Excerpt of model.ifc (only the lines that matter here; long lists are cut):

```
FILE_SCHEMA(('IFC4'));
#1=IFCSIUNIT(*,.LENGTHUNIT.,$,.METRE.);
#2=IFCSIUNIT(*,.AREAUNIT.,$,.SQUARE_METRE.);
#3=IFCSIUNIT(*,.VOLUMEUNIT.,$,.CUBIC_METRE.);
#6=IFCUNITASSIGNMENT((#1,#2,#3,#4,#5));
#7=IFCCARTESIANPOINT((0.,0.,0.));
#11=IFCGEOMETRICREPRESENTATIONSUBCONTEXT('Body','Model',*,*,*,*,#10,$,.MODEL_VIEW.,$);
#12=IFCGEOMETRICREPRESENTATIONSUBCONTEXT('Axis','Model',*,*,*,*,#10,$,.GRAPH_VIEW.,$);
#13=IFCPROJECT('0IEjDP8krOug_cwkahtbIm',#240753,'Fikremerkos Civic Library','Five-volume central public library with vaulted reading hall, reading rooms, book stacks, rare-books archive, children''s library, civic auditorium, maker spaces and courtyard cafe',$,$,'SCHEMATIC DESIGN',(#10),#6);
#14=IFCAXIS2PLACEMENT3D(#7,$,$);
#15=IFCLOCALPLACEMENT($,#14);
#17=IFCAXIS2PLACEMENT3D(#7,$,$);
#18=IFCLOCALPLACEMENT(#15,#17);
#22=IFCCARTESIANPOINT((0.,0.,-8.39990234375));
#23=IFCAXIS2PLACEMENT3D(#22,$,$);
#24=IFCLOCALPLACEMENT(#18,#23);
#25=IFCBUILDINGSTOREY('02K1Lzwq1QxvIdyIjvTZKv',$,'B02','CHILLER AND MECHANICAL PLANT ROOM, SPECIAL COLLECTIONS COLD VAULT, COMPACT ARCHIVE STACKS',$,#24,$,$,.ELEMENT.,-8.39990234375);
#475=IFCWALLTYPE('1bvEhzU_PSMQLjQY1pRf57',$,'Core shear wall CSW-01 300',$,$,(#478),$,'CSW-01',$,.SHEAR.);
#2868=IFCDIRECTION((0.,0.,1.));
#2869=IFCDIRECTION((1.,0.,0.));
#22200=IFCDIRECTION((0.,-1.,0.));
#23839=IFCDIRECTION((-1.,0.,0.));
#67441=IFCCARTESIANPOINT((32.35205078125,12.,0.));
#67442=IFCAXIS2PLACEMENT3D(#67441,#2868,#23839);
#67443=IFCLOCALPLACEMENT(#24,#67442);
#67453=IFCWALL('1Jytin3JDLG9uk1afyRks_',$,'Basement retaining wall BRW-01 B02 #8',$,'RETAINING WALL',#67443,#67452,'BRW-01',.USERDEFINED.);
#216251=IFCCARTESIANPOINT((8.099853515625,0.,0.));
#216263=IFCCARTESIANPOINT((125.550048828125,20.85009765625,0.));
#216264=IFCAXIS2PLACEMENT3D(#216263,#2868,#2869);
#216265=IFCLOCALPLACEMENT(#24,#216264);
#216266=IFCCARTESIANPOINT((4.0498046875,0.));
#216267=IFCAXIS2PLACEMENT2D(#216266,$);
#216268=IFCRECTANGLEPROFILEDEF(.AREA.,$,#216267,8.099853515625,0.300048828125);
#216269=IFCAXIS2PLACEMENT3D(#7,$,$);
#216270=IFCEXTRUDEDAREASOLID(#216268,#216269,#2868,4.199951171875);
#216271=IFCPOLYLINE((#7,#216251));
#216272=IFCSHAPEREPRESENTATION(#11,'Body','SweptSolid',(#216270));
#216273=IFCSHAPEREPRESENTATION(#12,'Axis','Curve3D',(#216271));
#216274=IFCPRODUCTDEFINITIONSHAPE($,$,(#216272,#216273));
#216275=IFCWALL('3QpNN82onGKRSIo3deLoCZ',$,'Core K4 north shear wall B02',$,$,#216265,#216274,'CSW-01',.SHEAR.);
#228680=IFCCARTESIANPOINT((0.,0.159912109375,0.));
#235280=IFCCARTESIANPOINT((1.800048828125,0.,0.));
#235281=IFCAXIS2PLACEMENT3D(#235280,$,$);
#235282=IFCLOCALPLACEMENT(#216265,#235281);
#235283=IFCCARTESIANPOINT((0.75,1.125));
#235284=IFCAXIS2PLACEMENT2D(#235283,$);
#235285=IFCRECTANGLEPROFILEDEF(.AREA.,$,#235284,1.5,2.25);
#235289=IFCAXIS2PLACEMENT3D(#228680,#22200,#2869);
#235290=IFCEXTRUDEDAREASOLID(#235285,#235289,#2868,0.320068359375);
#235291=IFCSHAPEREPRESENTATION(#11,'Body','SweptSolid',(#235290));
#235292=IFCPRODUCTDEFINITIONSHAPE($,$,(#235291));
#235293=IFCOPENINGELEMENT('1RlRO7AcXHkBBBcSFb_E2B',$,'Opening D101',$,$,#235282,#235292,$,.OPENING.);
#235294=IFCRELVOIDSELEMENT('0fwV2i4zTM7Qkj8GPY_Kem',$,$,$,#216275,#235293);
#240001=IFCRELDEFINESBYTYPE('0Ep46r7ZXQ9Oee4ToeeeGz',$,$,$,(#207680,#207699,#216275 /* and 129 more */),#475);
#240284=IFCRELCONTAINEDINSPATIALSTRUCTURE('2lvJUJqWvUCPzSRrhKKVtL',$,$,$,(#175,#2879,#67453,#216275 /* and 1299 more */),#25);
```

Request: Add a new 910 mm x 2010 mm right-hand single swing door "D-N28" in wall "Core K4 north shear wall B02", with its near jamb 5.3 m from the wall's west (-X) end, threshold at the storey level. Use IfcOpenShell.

```python
import numpy as np
import ifcopenshell
import ifcopenshell.api.feature
import ifcopenshell.api.geometry
import ifcopenshell.api.root
import ifcopenshell.api.spatial
import ifcopenshell.geom
import ifcopenshell.util.element
import ifcopenshell.util.placement
import ifcopenshell.util.representation
import ifcopenshell.util.shape
import ifcopenshell.util.unit

model = ifcopenshell.open("model.ifc")
unit_scale = ifcopenshell.util.unit.calculate_unit_scale(model)
settings = ifcopenshell.geom.settings()


def volume(element):
    """Net volume in cubic metres, openings subtracted."""
    shape = ifcopenshell.geom.create_shape(settings, element)
    return ifcopenshell.util.shape.get_volume(shape.geometry)


wall = model.by_guid("3QpNN82onGKRSIo3deLoCZ")
storey = ifcopenshell.util.element.get_container(wall, ifc_class="IfcBuildingStorey")
context = ifcopenshell.util.representation.get_context(model, "Model", "Body", "MODEL_VIEW")
before = volume(wall)

width, height, from_end, sill = 0.91, 2.01, 5.3, 0.0  # metres

# The wall runs along its own X axis, and the end named is its -X end.
wall_shape = ifcopenshell.geom.create_shape(settings, wall)
x, y, z = ifcopenshell.util.shape.get_vertices(wall_shape.geometry).T
start = x.min() + from_end
face, thickness = float(y.min()), float(y.max() - y.min())
wall_matrix = ifcopenshell.util.placement.get_local_placement(wall.ObjectPlacement)
level = ifcopenshell.util.placement.get_local_placement(storey.ObjectPlacement)[2, 3]


def in_wall(x, y):
    """Placement at x, y metres in the wall's axes, at sill height."""
    matrix = wall_matrix.copy()
    matrix[:, 3] = wall_matrix @ np.array([x / unit_scale, y / unit_scale, 0.0, 1.0])
    matrix[2, 3] = level + sill / unit_scale
    return matrix


# Opening: a box that overshoots both wall faces by 50 mm.
opening = ifcopenshell.api.root.create_entity(model, ifc_class="IfcOpeningElement", predefined_type="OPENING")
box = ifcopenshell.api.geometry.add_wall_representation(
    model, context=context, length=width, height=height, thickness=thickness + 0.1
)
ifcopenshell.api.geometry.assign_representation(model, product=opening, representation=box)
ifcopenshell.api.geometry.edit_object_placement(model, product=opening, matrix=in_wall(start, face - 0.05), is_si=False)
ifcopenshell.api.feature.add_feature(model, feature=opening, element=wall)

door = ifcopenshell.api.root.create_entity(model, ifc_class="IfcDoor", name="D-N28", predefined_type="DOOR")
door.OverallWidth, door.OverallHeight = width / unit_scale, height / unit_scale
door.OperationType = "SINGLE_SWING_RIGHT"
body = ifcopenshell.api.geometry.add_door_representation(
    model,
    context=context,
    overall_width=door.OverallWidth,
    overall_height=door.OverallHeight,
    operation_type="SINGLE_SWING_RIGHT",
    lining_properties={"LiningDepth": thickness / unit_scale, "ThresholdDepth": thickness / unit_scale},
)
ifcopenshell.api.geometry.assign_representation(model, product=door, representation=body)
ifcopenshell.api.spatial.assign_container(model, products=[door], relating_structure=storey)
ifcopenshell.api.feature.add_filling(model, opening=opening, element=door)

# The lining spans the wall, so the door starts at the wall face.
ifcopenshell.api.geometry.edit_object_placement(model, product=door, matrix=in_wall(start, face), is_si=False)

after = volume(wall)

print(f"wall volume {before:.3f} -> {after:.3f} m3")

model.write("model_rev.ifc")
```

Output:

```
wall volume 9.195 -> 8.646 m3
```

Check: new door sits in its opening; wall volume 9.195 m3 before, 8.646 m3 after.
